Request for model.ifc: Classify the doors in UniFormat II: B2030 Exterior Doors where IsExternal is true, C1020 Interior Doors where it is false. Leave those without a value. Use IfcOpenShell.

First a look at what the model holds.

```python
import ifcopenshell
import ifcopenshell.util.element

model = ifcopenshell.open("model.ifc")
print(model.schema)
print("classifications:", [c.Name for c in model.by_type("IfcClassification")])
values = [ifcopenshell.util.element.get_pset(e, "Pset_DoorCommon", "IsExternal") for e in model.by_type("IfcDoor")]
for value in (True, False, None):
    print("IsExternal", value, values.count(value))
```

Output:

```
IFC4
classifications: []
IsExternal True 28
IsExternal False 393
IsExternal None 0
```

```python
import ifcopenshell
import ifcopenshell.api.classification
import ifcopenshell.util.element

model = ifcopenshell.open("model.ifc")

system = ifcopenshell.api.classification.add_classification(model, classification="UniFormat II")

doors = model.by_type("IfcDoor")
external = {e: ifcopenshell.util.element.get_pset(e, "Pset_DoorCommon", "IsExternal") for e in doors}
for flag, code, name in ((True, "B2030", "Exterior Doors"), (False, "C1020", "Interior Doors")):
    products = [e for e in doors if external[e] is flag]
    ifcopenshell.api.classification.add_reference(
        model, products=products, classification=system, identification=code, name=name
    )
    print(code, len(products))

model.write("model_updated.ifc")
```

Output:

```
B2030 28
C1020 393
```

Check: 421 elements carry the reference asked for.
